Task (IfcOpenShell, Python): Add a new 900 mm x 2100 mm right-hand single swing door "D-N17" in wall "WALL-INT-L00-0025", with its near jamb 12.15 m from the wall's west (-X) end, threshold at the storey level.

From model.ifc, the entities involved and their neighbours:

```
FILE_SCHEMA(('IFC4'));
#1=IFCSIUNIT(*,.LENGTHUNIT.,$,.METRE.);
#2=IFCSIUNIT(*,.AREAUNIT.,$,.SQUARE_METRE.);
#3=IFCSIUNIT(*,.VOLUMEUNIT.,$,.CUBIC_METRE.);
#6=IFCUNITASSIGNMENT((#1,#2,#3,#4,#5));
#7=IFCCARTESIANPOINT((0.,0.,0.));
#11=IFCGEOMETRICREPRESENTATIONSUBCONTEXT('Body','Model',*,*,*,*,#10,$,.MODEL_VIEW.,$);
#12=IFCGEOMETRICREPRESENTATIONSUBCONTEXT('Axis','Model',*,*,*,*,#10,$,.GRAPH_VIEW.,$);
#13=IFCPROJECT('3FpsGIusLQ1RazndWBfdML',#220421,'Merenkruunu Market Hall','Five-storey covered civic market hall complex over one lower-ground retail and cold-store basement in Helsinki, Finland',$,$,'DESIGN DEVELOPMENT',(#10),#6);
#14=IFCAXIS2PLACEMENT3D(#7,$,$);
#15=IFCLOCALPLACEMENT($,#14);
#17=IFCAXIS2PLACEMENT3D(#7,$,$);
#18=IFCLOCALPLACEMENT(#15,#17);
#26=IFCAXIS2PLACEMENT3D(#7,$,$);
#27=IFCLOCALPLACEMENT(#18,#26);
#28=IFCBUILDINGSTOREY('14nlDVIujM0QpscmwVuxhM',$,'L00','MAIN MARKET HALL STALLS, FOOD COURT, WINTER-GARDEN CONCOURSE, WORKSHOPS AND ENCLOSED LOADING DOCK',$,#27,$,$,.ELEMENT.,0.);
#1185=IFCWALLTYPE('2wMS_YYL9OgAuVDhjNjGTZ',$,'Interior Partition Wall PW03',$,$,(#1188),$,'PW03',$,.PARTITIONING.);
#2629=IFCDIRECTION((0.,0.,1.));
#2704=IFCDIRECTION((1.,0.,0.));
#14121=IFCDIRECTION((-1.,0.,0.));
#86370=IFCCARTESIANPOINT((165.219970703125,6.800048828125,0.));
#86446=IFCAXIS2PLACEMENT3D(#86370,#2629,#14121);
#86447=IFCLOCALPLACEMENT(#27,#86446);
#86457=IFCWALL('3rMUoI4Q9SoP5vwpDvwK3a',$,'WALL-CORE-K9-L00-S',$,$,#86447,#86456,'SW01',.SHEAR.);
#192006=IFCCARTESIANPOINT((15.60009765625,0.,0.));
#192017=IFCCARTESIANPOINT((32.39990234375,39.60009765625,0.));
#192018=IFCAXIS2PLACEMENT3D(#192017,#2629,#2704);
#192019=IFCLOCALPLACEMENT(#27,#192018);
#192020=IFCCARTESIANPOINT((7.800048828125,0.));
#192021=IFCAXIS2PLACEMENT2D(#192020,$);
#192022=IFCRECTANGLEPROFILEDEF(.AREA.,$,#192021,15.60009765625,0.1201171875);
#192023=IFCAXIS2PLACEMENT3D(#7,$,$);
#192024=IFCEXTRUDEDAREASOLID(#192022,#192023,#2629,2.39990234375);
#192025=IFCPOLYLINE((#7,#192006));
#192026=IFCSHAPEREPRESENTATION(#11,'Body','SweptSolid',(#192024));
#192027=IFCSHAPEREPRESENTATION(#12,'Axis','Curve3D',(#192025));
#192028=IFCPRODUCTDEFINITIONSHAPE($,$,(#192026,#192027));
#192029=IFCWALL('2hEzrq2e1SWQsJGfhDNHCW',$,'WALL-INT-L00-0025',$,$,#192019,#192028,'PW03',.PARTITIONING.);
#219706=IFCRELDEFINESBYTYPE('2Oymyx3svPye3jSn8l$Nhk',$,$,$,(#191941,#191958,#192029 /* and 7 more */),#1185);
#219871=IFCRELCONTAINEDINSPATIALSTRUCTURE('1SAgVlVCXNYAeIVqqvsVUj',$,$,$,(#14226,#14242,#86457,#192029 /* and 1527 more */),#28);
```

```python
import numpy as np
import ifcopenshell
import ifcopenshell.api.feature
import ifcopenshell.api.geometry
import ifcopenshell.api.root
import ifcopenshell.api.spatial
import ifcopenshell.geom
import ifcopenshell.util.element
import ifcopenshell.util.placement
import ifcopenshell.util.representation
import ifcopenshell.util.shape
import ifcopenshell.util.unit

model = ifcopenshell.open("model.ifc")
unit_scale = ifcopenshell.util.unit.calculate_unit_scale(model)
settings = ifcopenshell.geom.settings()


def volume(element):
    """Net volume in cubic metres, openings subtracted."""
    shape = ifcopenshell.geom.create_shape(settings, element)
    return ifcopenshell.util.shape.get_volume(shape.geometry)


wall = model.by_guid("2hEzrq2e1SWQsJGfhDNHCW")
storey = ifcopenshell.util.element.get_container(wall, ifc_class="IfcBuildingStorey")
context = ifcopenshell.util.representation.get_context(model, "Model", "Body", "MODEL_VIEW")
before = volume(wall)

width, height, from_end, sill = 0.9, 2.1, 12.15, 0.0  # metres

# The wall runs along its own X axis, and the end named is its -X end.
wall_shape = ifcopenshell.geom.create_shape(settings, wall)
x, y, z = ifcopenshell.util.shape.get_vertices(wall_shape.geometry).T
start = x.min() + from_end
face, thickness = float(y.min()), float(y.max() - y.min())
wall_matrix = ifcopenshell.util.placement.get_local_placement(wall.ObjectPlacement)
level = ifcopenshell.util.placement.get_local_placement(storey.ObjectPlacement)[2, 3]


def in_wall(x, y):
    """Placement at x, y metres in the wall's axes, at sill height."""
    matrix = wall_matrix.copy()
    matrix[:, 3] = wall_matrix @ np.array([x / unit_scale, y / unit_scale, 0.0, 1.0])
    matrix[2, 3] = level + sill / unit_scale
    return matrix


# Opening: a box that overshoots both wall faces by 50 mm.
opening = ifcopenshell.api.root.create_entity(model, ifc_class="IfcOpeningElement", predefined_type="OPENING")
box = ifcopenshell.api.geometry.add_wall_representation(
    model, context=context, length=width, height=height, thickness=thickness + 0.1
)
ifcopenshell.api.geometry.assign_representation(model, product=opening, representation=box)
ifcopenshell.api.geometry.edit_object_placement(model, product=opening, matrix=in_wall(start, face - 0.05), is_si=False)
ifcopenshell.api.feature.add_feature(model, feature=opening, element=wall)

door = ifcopenshell.api.root.create_entity(model, ifc_class="IfcDoor", name="D-N17", predefined_type="DOOR")
door.OverallWidth, door.OverallHeight = width / unit_scale, height / unit_scale
door.OperationType = "SINGLE_SWING_RIGHT"
body = ifcopenshell.api.geometry.add_door_representation(
    model,
    context=context,
    overall_width=door.OverallWidth,
    overall_height=door.OverallHeight,
    operation_type="SINGLE_SWING_RIGHT",
    lining_properties={"LiningDepth": thickness / unit_scale, "ThresholdDepth": thickness / unit_scale},
)
ifcopenshell.api.geometry.assign_representation(model, product=door, representation=body)
ifcopenshell.api.spatial.assign_container(model, products=[door], relating_structure=storey)
ifcopenshell.api.feature.add_filling(model, opening=opening, element=door)

# The lining spans the wall, so the door starts at the wall face.
ifcopenshell.api.geometry.edit_object_placement(model, product=door, matrix=in_wall(start, face), is_si=False)

after = volume(wall)

print(f"wall volume {before:.3f} -> {after:.3f} m3")

model.write("model_updated.ifc")
```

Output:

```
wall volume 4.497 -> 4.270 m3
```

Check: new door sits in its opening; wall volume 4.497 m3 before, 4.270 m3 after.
